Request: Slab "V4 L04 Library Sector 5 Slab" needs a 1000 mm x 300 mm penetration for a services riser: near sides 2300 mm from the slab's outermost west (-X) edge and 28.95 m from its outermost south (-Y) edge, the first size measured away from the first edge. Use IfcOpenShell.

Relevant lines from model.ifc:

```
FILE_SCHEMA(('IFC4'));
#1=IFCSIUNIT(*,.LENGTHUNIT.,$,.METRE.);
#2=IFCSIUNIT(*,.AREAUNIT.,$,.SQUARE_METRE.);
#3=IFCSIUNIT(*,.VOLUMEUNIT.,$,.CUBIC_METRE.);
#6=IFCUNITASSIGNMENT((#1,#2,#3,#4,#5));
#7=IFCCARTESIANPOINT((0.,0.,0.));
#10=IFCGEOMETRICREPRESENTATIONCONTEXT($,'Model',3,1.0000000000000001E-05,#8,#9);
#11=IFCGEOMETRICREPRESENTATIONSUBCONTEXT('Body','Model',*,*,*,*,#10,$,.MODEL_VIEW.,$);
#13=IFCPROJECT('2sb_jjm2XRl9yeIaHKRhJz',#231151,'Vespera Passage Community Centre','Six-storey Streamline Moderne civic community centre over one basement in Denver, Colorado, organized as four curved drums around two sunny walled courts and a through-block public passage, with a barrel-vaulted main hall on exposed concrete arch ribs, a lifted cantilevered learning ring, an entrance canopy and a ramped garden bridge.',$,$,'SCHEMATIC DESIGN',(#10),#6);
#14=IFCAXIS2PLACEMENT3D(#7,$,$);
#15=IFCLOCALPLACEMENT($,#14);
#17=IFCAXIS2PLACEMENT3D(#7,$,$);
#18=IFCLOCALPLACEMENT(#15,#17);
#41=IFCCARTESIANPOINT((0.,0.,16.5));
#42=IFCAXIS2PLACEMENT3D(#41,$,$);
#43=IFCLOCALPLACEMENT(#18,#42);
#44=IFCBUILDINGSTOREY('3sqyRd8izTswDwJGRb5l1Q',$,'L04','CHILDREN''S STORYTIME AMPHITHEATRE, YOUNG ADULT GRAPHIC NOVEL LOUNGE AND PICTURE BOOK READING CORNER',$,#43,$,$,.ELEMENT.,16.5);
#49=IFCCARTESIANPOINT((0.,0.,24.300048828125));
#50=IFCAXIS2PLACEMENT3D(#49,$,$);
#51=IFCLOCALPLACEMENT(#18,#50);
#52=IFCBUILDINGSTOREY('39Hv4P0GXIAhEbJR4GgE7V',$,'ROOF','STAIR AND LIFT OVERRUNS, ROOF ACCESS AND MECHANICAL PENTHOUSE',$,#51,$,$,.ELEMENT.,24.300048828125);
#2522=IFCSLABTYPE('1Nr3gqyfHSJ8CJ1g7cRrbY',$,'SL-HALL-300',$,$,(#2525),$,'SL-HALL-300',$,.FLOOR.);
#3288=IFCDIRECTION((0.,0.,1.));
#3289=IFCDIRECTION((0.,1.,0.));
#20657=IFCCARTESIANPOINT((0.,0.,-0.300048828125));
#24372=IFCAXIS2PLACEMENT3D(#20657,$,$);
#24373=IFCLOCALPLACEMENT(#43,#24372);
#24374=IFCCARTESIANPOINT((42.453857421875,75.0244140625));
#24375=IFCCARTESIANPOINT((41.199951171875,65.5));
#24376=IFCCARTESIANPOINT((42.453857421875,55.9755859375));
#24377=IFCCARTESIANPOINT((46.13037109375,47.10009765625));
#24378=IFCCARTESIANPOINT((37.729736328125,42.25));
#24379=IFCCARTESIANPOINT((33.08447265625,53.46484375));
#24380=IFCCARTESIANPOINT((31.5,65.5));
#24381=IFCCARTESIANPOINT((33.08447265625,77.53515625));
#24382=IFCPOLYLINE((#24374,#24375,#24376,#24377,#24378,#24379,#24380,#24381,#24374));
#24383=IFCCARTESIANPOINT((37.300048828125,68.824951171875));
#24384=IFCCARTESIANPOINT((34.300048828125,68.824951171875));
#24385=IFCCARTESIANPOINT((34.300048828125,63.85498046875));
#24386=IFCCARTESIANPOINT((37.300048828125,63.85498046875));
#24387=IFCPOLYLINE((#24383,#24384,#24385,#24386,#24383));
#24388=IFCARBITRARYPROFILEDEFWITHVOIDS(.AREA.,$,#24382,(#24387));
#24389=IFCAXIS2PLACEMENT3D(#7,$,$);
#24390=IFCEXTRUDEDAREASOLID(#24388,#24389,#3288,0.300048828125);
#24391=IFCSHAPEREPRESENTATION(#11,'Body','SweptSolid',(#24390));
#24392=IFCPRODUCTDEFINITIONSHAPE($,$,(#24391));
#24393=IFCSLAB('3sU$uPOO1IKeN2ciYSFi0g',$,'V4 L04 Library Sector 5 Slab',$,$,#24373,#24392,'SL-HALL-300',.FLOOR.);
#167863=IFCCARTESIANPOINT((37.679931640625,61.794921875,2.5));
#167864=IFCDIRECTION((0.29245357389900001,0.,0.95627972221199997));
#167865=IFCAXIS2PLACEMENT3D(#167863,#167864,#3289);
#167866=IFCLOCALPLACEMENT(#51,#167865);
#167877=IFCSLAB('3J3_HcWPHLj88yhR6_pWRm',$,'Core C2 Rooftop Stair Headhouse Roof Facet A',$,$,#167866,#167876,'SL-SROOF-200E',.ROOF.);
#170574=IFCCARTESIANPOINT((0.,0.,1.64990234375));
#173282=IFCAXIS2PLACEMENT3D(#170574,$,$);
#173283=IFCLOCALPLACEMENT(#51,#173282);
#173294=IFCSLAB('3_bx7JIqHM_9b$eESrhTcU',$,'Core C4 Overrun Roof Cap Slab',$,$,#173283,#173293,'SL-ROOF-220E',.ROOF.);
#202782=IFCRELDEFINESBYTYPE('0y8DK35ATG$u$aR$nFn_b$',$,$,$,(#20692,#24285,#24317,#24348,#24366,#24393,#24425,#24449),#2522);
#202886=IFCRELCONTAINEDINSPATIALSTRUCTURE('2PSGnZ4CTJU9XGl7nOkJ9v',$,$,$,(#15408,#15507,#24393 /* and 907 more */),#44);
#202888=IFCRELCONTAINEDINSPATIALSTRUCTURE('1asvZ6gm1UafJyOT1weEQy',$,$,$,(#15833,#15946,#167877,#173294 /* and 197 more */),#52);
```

```python
import numpy as np
import ifcopenshell
import ifcopenshell.api.feature
import ifcopenshell.api.geometry
import ifcopenshell.api.root
import ifcopenshell.geom
import ifcopenshell.util.placement
import ifcopenshell.util.representation
import ifcopenshell.util.shape
import ifcopenshell.util.unit

model = ifcopenshell.open("model.ifc")
unit_scale = ifcopenshell.util.unit.calculate_unit_scale(model)
settings = ifcopenshell.geom.settings()


def volume(element):
    """Net volume in cubic metres, openings subtracted."""
    shape = ifcopenshell.geom.create_shape(settings, element)
    return ifcopenshell.util.shape.get_volume(shape.geometry)


slab = model.by_guid("3sU$uPOO1IKeN2ciYSFi0g")
before = volume(slab)

# Extent in the slab's own axes, in metres. The edges named are its -X and -Y sides.
slab_shape = ifcopenshell.geom.create_shape(settings, slab)
vertices = ifcopenshell.util.shape.get_vertices(slab_shape.geometry)
x_min, y_min, bottom = vertices.min(axis=0)
top = vertices[:, 2].max()

opening = ifcopenshell.api.root.create_entity(model, ifc_class="IfcOpeningElement", name="Services riser opening", predefined_type="OPENING")
context = ifcopenshell.util.representation.get_context(model, "Model", "Body", "MODEL_VIEW")
width, depth = 1, 0.3
outline = [(0.0, 0.0), (width, 0.0), (width, depth), (0.0, depth), (0.0, 0.0)]
# Overshoot both faces by 50 mm so the cut is clean.
shape = ifcopenshell.api.geometry.add_slab_representation(
    model, context=context, depth=top - bottom + 0.1, polyline=outline
)
ifcopenshell.api.geometry.assign_representation(model, product=opening, representation=shape)

matrix = ifcopenshell.util.placement.get_local_placement(slab.ObjectPlacement)
matrix[:, 3] = matrix @ np.append(np.array([x_min + 2.3, y_min + 28.95, bottom - 0.05]) / unit_scale, 1.0)
ifcopenshell.api.geometry.edit_object_placement(model, product=opening, matrix=matrix, is_si=False)
ifcopenshell.api.feature.add_feature(model, feature=opening, element=slab)

after = volume(slab)

print(f"slab volume {before:.3f} -> {after:.3f} m3")

model.write("model_rev.ifc")
```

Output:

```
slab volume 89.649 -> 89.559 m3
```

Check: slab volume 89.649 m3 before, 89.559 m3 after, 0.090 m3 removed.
